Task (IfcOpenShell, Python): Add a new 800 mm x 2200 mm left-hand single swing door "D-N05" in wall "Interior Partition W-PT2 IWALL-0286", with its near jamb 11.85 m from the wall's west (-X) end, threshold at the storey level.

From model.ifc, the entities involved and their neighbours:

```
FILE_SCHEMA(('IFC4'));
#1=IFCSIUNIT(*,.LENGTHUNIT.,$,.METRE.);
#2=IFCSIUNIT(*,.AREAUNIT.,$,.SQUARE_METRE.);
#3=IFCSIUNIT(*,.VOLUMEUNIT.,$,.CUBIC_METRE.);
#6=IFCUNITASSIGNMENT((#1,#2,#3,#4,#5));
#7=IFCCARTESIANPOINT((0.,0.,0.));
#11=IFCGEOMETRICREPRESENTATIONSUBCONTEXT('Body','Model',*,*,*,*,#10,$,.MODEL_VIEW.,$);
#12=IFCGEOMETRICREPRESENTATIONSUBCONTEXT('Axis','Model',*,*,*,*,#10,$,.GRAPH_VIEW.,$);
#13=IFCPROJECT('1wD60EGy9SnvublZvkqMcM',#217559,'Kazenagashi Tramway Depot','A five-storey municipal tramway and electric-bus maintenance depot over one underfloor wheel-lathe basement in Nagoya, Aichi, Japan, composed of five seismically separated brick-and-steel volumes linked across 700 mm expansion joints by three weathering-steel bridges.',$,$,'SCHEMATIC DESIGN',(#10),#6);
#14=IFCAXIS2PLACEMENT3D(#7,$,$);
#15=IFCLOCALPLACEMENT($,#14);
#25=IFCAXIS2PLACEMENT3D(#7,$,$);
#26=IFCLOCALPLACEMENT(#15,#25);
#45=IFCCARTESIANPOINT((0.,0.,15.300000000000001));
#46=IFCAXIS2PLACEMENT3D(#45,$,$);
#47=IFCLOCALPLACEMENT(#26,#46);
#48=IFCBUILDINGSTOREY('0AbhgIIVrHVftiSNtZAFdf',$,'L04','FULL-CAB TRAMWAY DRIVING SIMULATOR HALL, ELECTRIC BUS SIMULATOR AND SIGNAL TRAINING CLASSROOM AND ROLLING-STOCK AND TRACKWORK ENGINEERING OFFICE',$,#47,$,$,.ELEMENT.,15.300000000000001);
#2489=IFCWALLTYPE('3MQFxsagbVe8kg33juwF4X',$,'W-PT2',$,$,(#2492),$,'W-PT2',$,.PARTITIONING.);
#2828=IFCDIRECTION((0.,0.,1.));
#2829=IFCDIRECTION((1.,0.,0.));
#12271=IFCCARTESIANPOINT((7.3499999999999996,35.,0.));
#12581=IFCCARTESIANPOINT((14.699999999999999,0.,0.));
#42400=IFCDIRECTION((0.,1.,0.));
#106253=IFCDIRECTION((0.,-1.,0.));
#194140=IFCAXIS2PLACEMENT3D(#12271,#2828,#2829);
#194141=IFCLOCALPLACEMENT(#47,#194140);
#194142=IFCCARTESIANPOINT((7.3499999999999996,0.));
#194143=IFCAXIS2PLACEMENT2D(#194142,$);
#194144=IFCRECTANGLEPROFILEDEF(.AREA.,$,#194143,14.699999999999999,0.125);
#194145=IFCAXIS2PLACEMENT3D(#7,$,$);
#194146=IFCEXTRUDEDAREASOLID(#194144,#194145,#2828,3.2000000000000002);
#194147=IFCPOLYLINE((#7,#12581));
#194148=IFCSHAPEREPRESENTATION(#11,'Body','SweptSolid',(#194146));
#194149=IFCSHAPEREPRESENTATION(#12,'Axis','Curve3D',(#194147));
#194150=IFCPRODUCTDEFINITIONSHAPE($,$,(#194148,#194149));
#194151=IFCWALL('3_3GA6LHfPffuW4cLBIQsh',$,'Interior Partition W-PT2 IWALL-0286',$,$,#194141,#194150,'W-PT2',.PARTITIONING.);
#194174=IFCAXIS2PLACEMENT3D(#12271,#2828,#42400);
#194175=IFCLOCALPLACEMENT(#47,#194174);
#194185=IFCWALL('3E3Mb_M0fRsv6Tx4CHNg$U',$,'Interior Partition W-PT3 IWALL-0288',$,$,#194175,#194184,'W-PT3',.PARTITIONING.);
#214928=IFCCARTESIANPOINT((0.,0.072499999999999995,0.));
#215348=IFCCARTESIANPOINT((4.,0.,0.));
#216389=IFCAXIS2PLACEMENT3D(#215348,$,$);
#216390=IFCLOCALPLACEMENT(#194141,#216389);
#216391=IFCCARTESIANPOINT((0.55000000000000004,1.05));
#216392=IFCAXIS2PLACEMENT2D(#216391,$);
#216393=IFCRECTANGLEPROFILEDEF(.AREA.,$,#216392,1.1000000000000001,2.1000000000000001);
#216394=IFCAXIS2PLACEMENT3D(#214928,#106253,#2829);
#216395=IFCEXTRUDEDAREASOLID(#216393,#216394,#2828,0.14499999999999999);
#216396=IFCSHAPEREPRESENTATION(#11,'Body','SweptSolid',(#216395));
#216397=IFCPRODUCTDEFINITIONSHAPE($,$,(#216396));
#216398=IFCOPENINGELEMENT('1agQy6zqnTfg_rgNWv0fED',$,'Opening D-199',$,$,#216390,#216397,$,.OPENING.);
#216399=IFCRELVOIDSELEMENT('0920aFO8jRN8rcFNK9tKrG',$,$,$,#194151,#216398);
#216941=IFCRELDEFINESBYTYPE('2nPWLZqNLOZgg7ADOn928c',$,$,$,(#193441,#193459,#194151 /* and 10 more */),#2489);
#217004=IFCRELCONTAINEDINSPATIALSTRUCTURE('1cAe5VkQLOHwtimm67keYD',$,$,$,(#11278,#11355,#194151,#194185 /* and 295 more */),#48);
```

```python
import numpy as np
import ifcopenshell
import ifcopenshell.api.feature
import ifcopenshell.api.geometry
import ifcopenshell.api.root
import ifcopenshell.api.spatial
import ifcopenshell.geom
import ifcopenshell.util.element
import ifcopenshell.util.placement
import ifcopenshell.util.representation
import ifcopenshell.util.shape
import ifcopenshell.util.unit

model = ifcopenshell.open("model.ifc")
unit_scale = ifcopenshell.util.unit.calculate_unit_scale(model)
settings = ifcopenshell.geom.settings()


def volume(element):
    """Net volume in cubic metres, openings subtracted."""
    shape = ifcopenshell.geom.create_shape(settings, element)
    return ifcopenshell.util.shape.get_volume(shape.geometry)


wall = model.by_guid("3_3GA6LHfPffuW4cLBIQsh")
storey = ifcopenshell.util.element.get_container(wall, ifc_class="IfcBuildingStorey")
context = ifcopenshell.util.representation.get_context(model, "Model", "Body", "MODEL_VIEW")
before = volume(wall)

width, height, from_end, sill = 0.8, 2.2, 11.85, 0.0  # metres

# The wall runs along its own X axis, and the end named is its -X end.
wall_shape = ifcopenshell.geom.create_shape(settings, wall)
x, y, z = ifcopenshell.util.shape.get_vertices(wall_shape.geometry).T
start = x.min() + from_end
face, thickness = float(y.min()), float(y.max() - y.min())
wall_matrix = ifcopenshell.util.placement.get_local_placement(wall.ObjectPlacement)
level = ifcopenshell.util.placement.get_local_placement(storey.ObjectPlacement)[2, 3]


def in_wall(x, y):
    """Placement at x, y metres in the wall's axes, at sill height."""
    matrix = wall_matrix.copy()
    matrix[:, 3] = wall_matrix @ np.array([x / unit_scale, y / unit_scale, 0.0, 1.0])
    matrix[2, 3] = level + sill / unit_scale
    return matrix


# Opening: a box that overshoots both wall faces by 50 mm.
opening = ifcopenshell.api.root.create_entity(model, ifc_class="IfcOpeningElement", predefined_type="OPENING")
box = ifcopenshell.api.geometry.add_wall_representation(
    model, context=context, length=width, height=height, thickness=thickness + 0.1
)
ifcopenshell.api.geometry.assign_representation(model, product=opening, representation=box)
ifcopenshell.api.geometry.edit_object_placement(model, product=opening, matrix=in_wall(start, face - 0.05), is_si=False)
ifcopenshell.api.feature.add_feature(model, feature=opening, element=wall)

door = ifcopenshell.api.root.create_entity(model, ifc_class="IfcDoor", name="D-N05", predefined_type="DOOR")
door.OverallWidth, door.OverallHeight = width / unit_scale, height / unit_scale
door.OperationType = "SINGLE_SWING_LEFT"
body = ifcopenshell.api.geometry.add_door_representation(
    model,
    context=context,
    overall_width=door.OverallWidth,
    overall_height=door.OverallHeight,
    operation_type="SINGLE_SWING_LEFT",
    lining_properties={"LiningDepth": thickness / unit_scale, "ThresholdDepth": thickness / unit_scale},
)
ifcopenshell.api.geometry.assign_representation(model, product=door, representation=body)
ifcopenshell.api.spatial.assign_container(model, products=[door], relating_structure=storey)
ifcopenshell.api.feature.add_filling(model, opening=opening, element=door)

# The lining spans the wall, so the door starts at the wall face.
ifcopenshell.api.geometry.edit_object_placement(model, product=door, matrix=in_wall(start, face), is_si=False)

after = volume(wall)

print(f"wall volume {before:.3f} -> {after:.3f} m3")

model.write("model_v2.ifc")
```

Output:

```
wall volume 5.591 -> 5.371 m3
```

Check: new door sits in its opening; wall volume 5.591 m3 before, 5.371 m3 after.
